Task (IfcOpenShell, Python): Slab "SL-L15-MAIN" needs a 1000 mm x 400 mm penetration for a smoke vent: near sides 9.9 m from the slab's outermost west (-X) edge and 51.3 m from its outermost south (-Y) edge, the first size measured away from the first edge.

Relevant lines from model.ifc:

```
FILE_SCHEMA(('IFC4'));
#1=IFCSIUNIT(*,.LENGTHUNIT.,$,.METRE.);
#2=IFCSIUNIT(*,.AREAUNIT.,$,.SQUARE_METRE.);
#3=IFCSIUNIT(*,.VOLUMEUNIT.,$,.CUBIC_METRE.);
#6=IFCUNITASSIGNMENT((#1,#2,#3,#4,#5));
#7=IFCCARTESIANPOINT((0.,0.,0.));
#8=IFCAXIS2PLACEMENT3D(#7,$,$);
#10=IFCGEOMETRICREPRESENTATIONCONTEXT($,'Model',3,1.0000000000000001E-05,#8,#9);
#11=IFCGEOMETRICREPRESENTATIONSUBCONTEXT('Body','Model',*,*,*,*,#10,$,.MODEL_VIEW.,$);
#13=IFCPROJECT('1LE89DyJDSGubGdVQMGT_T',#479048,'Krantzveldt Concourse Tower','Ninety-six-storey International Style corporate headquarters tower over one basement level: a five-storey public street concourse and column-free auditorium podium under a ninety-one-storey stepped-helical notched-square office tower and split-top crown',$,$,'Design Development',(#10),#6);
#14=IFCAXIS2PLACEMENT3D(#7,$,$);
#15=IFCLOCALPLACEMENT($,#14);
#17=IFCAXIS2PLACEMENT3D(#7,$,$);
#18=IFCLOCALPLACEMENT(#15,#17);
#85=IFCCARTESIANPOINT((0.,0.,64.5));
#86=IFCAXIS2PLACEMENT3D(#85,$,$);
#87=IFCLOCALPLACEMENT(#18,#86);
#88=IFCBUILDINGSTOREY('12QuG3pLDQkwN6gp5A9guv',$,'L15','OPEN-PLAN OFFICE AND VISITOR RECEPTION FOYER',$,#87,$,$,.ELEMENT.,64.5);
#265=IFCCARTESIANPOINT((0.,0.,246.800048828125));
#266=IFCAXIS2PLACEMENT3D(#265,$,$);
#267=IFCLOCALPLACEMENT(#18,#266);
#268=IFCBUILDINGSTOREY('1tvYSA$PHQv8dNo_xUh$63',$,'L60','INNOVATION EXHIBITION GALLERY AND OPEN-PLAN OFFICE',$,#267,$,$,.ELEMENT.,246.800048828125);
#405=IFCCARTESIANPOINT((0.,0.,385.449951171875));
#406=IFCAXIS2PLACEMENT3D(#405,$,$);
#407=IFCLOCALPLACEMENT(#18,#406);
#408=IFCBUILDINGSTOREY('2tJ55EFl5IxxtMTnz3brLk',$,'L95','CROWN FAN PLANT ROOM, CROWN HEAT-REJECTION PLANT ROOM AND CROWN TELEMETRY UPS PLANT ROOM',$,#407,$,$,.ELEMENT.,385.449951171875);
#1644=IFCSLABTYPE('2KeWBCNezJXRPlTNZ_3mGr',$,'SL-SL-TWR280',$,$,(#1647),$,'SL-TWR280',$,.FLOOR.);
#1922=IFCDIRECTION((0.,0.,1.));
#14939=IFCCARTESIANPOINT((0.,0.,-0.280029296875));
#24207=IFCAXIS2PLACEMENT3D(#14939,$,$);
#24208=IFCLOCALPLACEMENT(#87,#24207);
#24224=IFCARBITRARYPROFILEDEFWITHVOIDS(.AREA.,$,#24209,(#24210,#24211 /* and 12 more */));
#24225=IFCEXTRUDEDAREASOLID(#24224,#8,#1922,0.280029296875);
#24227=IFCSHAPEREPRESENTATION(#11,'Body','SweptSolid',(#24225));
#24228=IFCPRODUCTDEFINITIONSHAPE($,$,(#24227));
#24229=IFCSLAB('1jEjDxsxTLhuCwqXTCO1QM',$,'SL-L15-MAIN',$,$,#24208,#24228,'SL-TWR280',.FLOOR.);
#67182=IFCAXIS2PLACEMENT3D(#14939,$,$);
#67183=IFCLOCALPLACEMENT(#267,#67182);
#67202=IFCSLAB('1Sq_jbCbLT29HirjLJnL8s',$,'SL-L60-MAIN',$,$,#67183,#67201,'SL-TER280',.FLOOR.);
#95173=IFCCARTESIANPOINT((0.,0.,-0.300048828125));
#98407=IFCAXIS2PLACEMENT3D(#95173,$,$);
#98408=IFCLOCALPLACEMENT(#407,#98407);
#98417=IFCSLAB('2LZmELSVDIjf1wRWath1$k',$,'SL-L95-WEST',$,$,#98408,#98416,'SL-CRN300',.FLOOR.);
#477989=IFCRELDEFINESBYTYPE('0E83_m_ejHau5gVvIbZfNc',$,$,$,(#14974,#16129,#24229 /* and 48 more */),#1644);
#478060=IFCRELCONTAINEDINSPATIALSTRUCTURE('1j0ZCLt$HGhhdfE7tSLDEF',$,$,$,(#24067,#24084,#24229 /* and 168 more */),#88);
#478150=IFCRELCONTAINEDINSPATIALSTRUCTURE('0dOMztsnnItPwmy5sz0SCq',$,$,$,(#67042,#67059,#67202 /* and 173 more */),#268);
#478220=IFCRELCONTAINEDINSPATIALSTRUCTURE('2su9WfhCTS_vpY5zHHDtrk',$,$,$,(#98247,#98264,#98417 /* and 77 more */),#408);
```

```python
import numpy as np
import ifcopenshell
import ifcopenshell.api.feature
import ifcopenshell.api.geometry
import ifcopenshell.api.root
import ifcopenshell.geom
import ifcopenshell.util.placement
import ifcopenshell.util.representation
import ifcopenshell.util.shape
import ifcopenshell.util.unit

model = ifcopenshell.open("model.ifc")
unit_scale = ifcopenshell.util.unit.calculate_unit_scale(model)
settings = ifcopenshell.geom.settings()


def volume(element):
    """Net volume in cubic metres, openings subtracted."""
    shape = ifcopenshell.geom.create_shape(settings, element)
    return ifcopenshell.util.shape.get_volume(shape.geometry)


slab = model.by_guid("1jEjDxsxTLhuCwqXTCO1QM")
before = volume(slab)

# Extent in the slab's own axes, in metres. The edges named are its -X and -Y sides.
slab_shape = ifcopenshell.geom.create_shape(settings, slab)
vertices = ifcopenshell.util.shape.get_vertices(slab_shape.geometry)
x_min, y_min, bottom = vertices.min(axis=0)
top = vertices[:, 2].max()

opening = ifcopenshell.api.root.create_entity(model, ifc_class="IfcOpeningElement", name="Smoke vent opening", predefined_type="OPENING")
context = ifcopenshell.util.representation.get_context(model, "Model", "Body", "MODEL_VIEW")
width, depth = 1, 0.4
outline = [(0.0, 0.0), (width, 0.0), (width, depth), (0.0, depth), (0.0, 0.0)]
# Overshoot both faces by 50 mm so the cut is clean.
shape = ifcopenshell.api.geometry.add_slab_representation(
    model, context=context, depth=top - bottom + 0.1, polyline=outline
)
ifcopenshell.api.geometry.assign_representation(model, product=opening, representation=shape)

matrix = ifcopenshell.util.placement.get_local_placement(slab.ObjectPlacement)
matrix[:, 3] = matrix @ np.append(np.array([x_min + 9.9, y_min + 51.3, bottom - 0.05]) / unit_scale, 1.0)
ifcopenshell.api.geometry.edit_object_placement(model, product=opening, matrix=matrix, is_si=False)
ifcopenshell.api.feature.add_feature(model, feature=opening, element=slab)

after = volume(slab)

print(f"slab volume {before:.3f} -> {after:.3f} m3")

model.write("model_edited.ifc")
```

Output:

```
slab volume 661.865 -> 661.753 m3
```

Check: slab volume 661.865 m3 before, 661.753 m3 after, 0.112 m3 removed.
